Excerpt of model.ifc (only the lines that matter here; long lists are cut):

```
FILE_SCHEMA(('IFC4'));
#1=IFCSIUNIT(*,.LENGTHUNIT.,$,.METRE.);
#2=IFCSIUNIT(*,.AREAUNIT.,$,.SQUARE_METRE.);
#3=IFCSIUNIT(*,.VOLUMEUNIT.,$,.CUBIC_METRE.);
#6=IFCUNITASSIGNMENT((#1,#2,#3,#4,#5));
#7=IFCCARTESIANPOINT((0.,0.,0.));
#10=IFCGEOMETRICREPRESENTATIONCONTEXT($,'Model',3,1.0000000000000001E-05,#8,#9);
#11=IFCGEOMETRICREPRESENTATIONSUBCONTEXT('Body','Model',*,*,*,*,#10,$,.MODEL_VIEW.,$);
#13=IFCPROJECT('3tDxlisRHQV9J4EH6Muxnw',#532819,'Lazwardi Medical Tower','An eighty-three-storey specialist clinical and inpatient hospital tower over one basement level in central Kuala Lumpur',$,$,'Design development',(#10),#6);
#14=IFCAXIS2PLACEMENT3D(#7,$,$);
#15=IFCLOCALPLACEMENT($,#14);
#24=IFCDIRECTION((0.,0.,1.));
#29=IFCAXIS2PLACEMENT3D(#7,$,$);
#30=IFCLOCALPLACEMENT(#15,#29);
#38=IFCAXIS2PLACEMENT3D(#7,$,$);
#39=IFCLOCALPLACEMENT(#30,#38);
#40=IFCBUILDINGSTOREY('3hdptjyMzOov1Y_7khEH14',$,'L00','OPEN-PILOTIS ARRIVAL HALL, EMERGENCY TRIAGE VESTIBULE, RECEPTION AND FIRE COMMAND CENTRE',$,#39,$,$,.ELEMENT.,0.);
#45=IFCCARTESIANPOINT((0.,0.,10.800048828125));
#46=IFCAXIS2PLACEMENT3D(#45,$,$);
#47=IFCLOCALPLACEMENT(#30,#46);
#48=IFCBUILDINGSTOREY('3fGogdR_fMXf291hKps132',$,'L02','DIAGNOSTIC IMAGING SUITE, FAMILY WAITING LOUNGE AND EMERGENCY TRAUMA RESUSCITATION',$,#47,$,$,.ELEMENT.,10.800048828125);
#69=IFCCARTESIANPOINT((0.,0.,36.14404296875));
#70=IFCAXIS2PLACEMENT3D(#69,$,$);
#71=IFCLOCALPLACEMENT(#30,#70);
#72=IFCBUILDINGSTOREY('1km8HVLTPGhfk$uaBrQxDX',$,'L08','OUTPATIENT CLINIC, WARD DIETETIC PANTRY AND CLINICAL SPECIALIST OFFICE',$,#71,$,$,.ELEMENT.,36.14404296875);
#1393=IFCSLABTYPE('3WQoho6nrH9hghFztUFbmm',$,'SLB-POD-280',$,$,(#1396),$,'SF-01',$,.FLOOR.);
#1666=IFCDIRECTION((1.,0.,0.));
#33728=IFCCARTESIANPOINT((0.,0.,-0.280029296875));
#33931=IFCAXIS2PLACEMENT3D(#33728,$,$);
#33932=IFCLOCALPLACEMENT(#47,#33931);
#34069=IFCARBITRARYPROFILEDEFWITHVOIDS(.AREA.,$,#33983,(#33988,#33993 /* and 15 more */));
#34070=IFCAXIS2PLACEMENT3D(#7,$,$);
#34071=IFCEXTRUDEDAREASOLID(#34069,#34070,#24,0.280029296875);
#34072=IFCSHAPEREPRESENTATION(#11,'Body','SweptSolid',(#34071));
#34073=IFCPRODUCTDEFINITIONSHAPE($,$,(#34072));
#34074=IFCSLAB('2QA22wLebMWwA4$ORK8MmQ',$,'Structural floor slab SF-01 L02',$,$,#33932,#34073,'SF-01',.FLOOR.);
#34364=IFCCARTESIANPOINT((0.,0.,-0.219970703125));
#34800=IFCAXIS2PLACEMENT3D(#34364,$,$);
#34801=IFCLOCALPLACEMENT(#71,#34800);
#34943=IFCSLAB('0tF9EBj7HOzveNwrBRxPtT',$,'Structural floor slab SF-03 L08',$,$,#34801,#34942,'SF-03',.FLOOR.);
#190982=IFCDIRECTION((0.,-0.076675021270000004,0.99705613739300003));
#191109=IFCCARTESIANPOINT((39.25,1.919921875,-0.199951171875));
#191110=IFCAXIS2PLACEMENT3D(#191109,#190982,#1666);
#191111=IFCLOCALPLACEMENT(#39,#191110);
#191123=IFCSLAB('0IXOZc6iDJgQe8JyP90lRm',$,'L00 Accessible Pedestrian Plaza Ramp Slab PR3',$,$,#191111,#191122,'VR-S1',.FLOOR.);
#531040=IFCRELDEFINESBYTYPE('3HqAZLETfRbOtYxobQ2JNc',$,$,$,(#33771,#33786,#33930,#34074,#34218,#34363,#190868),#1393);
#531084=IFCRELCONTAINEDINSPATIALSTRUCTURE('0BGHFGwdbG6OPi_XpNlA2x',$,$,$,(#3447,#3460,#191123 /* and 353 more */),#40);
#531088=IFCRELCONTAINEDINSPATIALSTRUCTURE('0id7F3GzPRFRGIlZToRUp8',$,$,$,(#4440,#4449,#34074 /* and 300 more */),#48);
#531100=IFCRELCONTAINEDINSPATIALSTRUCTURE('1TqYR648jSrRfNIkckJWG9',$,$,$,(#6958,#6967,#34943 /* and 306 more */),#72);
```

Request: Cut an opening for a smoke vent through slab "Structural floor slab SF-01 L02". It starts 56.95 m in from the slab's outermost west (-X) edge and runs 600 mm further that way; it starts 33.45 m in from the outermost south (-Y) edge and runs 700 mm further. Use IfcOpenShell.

```python
import numpy as np
import ifcopenshell
import ifcopenshell.api.feature
import ifcopenshell.api.geometry
import ifcopenshell.api.root
import ifcopenshell.geom
import ifcopenshell.util.placement
import ifcopenshell.util.representation
import ifcopenshell.util.shape
import ifcopenshell.util.unit

model = ifcopenshell.open("model.ifc")
unit_scale = ifcopenshell.util.unit.calculate_unit_scale(model)
settings = ifcopenshell.geom.settings()


def volume(element):
    """Net volume in cubic metres, openings subtracted."""
    shape = ifcopenshell.geom.create_shape(settings, element)
    return ifcopenshell.util.shape.get_volume(shape.geometry)


slab = model.by_guid("2QA22wLebMWwA4$ORK8MmQ")
before = volume(slab)

# Extent in the slab's own axes, in metres. The edges named are its -X and -Y sides.
slab_shape = ifcopenshell.geom.create_shape(settings, slab)
vertices = ifcopenshell.util.shape.get_vertices(slab_shape.geometry)
x_min, y_min, bottom = vertices.min(axis=0)
top = vertices[:, 2].max()

opening = ifcopenshell.api.root.create_entity(model, ifc_class="IfcOpeningElement", name="Smoke vent opening", predefined_type="OPENING")
context = ifcopenshell.util.representation.get_context(model, "Model", "Body", "MODEL_VIEW")
width, depth = 0.6, 0.7
outline = [(0.0, 0.0), (width, 0.0), (width, depth), (0.0, depth), (0.0, 0.0)]
# Overshoot both faces by 50 mm so the cut is clean.
shape = ifcopenshell.api.geometry.add_slab_representation(
    model, context=context, depth=top - bottom + 0.1, polyline=outline
)
ifcopenshell.api.geometry.assign_representation(model, product=opening, representation=shape)

matrix = ifcopenshell.util.placement.get_local_placement(slab.ObjectPlacement)
matrix[:, 3] = matrix @ np.append(np.array([x_min + 56.95, y_min + 33.45, bottom - 0.05]) / unit_scale, 1.0)
ifcopenshell.api.geometry.edit_object_placement(model, product=opening, matrix=matrix, is_si=False)
ifcopenshell.api.feature.add_feature(model, feature=opening, element=slab)

after = volume(slab)

print(f"slab volume {before:.3f} -> {after:.3f} m3")

model.write("model_rev.ifc")
```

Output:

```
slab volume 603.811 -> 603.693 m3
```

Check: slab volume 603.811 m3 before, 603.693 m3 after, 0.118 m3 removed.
